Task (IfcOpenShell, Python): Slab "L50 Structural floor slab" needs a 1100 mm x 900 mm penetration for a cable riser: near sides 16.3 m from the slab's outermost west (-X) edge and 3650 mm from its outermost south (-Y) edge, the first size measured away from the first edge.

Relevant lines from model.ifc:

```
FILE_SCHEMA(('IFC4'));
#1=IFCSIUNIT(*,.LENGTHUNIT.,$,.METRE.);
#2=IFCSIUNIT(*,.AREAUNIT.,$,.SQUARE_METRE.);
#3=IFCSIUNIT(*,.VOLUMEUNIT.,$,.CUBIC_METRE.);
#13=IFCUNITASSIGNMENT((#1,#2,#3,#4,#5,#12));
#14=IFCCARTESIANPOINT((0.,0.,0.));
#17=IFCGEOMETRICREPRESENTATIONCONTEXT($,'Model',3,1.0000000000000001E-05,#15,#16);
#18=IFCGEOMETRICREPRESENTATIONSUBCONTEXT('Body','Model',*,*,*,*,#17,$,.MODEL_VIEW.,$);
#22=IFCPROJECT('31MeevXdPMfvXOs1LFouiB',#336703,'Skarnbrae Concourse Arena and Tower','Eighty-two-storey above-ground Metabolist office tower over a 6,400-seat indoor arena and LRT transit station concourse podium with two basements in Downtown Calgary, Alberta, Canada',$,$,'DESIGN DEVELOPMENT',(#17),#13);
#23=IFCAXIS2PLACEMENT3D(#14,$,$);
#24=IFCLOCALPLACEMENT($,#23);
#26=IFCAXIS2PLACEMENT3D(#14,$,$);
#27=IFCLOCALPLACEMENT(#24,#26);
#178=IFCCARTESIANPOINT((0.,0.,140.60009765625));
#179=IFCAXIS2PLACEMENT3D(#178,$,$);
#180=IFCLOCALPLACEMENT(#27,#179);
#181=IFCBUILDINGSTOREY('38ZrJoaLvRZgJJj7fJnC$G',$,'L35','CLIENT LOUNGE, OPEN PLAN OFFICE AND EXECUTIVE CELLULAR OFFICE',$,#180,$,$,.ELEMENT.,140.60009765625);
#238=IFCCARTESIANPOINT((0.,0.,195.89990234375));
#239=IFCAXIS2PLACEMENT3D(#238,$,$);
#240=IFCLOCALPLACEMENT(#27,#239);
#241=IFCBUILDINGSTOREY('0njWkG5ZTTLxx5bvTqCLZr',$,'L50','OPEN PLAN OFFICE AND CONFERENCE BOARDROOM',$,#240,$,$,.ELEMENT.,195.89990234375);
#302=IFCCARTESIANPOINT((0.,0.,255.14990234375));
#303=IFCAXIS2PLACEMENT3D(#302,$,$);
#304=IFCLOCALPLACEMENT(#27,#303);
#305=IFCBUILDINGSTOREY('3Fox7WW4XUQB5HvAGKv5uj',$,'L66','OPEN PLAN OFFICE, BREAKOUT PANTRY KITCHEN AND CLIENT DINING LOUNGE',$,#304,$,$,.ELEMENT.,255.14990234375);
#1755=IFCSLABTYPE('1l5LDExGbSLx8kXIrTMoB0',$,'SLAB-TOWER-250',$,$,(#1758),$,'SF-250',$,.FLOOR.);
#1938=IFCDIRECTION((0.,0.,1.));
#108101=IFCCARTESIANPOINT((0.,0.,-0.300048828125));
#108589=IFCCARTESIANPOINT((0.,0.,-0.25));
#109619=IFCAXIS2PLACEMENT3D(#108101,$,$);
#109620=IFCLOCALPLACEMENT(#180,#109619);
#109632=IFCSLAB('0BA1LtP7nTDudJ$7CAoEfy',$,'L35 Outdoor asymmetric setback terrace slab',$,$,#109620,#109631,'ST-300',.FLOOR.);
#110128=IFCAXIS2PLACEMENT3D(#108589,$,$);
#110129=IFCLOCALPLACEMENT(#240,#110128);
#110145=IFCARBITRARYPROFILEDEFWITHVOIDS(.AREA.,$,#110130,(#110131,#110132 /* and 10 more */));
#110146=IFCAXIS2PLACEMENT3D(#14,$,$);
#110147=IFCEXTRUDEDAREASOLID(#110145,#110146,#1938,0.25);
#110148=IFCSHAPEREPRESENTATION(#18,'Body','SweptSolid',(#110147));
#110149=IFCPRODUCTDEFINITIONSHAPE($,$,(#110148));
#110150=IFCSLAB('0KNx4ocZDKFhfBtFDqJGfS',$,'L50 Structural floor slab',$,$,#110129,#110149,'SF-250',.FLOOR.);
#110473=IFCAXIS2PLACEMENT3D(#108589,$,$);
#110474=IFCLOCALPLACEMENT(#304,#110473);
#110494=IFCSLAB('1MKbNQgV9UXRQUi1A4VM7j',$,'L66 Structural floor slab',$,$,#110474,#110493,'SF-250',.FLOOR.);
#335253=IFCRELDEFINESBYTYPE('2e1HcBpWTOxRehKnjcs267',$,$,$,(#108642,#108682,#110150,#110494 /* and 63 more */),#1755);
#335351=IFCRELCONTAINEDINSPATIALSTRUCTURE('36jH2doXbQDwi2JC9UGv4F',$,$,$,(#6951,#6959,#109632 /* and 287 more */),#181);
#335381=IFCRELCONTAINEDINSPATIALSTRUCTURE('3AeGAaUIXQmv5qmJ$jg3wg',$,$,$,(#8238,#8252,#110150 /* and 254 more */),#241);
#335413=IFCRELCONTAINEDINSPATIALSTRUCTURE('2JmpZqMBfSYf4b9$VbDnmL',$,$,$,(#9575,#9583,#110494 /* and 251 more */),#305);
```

```python
import numpy as np
import ifcopenshell
import ifcopenshell.api.feature
import ifcopenshell.api.geometry
import ifcopenshell.api.root
import ifcopenshell.geom
import ifcopenshell.util.placement
import ifcopenshell.util.representation
import ifcopenshell.util.shape
import ifcopenshell.util.unit

model = ifcopenshell.open("model.ifc")
unit_scale = ifcopenshell.util.unit.calculate_unit_scale(model)
settings = ifcopenshell.geom.settings()


def volume(element):
    """Net volume in cubic metres, openings subtracted."""
    shape = ifcopenshell.geom.create_shape(settings, element)
    return ifcopenshell.util.shape.get_volume(shape.geometry)


slab = model.by_guid("0KNx4ocZDKFhfBtFDqJGfS")
before = volume(slab)

# Extent in the slab's own axes, in metres. The edges named are its -X and -Y sides.
slab_shape = ifcopenshell.geom.create_shape(settings, slab)
vertices = ifcopenshell.util.shape.get_vertices(slab_shape.geometry)
x_min, y_min, bottom = vertices.min(axis=0)
top = vertices[:, 2].max()

opening = ifcopenshell.api.root.create_entity(model, ifc_class="IfcOpeningElement", name="Cable riser opening", predefined_type="OPENING")
context = ifcopenshell.util.representation.get_context(model, "Model", "Body", "MODEL_VIEW")
width, depth = 1.1, 0.9
outline = [(0.0, 0.0), (width, 0.0), (width, depth), (0.0, depth), (0.0, 0.0)]
# Overshoot both faces by 50 mm so the cut is clean.
shape = ifcopenshell.api.geometry.add_slab_representation(
    model, context=context, depth=top - bottom + 0.1, polyline=outline
)
ifcopenshell.api.geometry.assign_representation(model, product=opening, representation=shape)

matrix = ifcopenshell.util.placement.get_local_placement(slab.ObjectPlacement)
matrix[:, 3] = matrix @ np.append(np.array([x_min + 16.3, y_min + 3.65, bottom - 0.05]) / unit_scale, 1.0)
ifcopenshell.api.geometry.edit_object_placement(model, product=opening, matrix=matrix, is_si=False)
ifcopenshell.api.feature.add_feature(model, feature=opening, element=slab)

after = volume(slab)

print(f"slab volume {before:.3f} -> {after:.3f} m3")

model.write("model_edited.ifc")
```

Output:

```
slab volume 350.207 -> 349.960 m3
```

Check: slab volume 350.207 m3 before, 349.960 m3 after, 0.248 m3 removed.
